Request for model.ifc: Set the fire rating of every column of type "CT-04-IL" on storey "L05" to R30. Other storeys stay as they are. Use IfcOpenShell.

First a look at what the model holds.

```python
import ifcopenshell
import ifcopenshell.util.element

model = ifcopenshell.open("model.ifc")
print(model.schema)
storey = next(s for s in model.by_type("IfcBuildingStorey") if s.Name == "L05")
columns = [e for e in ifcopenshell.util.element.get_decomposition(storey) if e.is_a("IfcColumn")]
seen = {}
for e in columns:
    element_type = ifcopenshell.util.element.get_type(e)
    key = (element_type.Name if element_type != e and element_type else None, ifcopenshell.util.element.get_pset(e, "Pset_ColumnCommon", "FireRating"))
    seen[key] = seen.get(key, 0) + 1
for (name, value), count in sorted(seen.items(), key=str):
    print(count, "x", name, "|", value)
```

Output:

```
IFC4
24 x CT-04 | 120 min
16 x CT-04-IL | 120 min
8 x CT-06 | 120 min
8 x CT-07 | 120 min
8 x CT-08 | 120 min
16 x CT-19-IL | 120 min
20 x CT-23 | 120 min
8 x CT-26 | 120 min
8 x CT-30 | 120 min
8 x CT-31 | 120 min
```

```python
import ifcopenshell
import ifcopenshell.api.pset
import ifcopenshell.util.element

model = ifcopenshell.open("model.ifc")

storey = next(s for s in model.by_type("IfcBuildingStorey") if s.Name == "L05")
columns = [e for e in ifcopenshell.util.element.get_decomposition(storey) if e.is_a("IfcColumn")]

count = 0
for e in columns:
    element_type = ifcopenshell.util.element.get_type(e)
    if element_type in (None, e) or element_type.Name != "CT-04-IL":
        continue
    # add_pset returns the element's existing set when there is one.
    pset = ifcopenshell.api.pset.add_pset(model, product=e, name="Pset_ColumnCommon")
    ifcopenshell.api.pset.edit_pset(model, pset=pset, properties={"FireRating": "R30"})
    count += 1

print(count, "columns updated")

model.write("model_updated.ifc")
```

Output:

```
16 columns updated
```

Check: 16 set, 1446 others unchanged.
